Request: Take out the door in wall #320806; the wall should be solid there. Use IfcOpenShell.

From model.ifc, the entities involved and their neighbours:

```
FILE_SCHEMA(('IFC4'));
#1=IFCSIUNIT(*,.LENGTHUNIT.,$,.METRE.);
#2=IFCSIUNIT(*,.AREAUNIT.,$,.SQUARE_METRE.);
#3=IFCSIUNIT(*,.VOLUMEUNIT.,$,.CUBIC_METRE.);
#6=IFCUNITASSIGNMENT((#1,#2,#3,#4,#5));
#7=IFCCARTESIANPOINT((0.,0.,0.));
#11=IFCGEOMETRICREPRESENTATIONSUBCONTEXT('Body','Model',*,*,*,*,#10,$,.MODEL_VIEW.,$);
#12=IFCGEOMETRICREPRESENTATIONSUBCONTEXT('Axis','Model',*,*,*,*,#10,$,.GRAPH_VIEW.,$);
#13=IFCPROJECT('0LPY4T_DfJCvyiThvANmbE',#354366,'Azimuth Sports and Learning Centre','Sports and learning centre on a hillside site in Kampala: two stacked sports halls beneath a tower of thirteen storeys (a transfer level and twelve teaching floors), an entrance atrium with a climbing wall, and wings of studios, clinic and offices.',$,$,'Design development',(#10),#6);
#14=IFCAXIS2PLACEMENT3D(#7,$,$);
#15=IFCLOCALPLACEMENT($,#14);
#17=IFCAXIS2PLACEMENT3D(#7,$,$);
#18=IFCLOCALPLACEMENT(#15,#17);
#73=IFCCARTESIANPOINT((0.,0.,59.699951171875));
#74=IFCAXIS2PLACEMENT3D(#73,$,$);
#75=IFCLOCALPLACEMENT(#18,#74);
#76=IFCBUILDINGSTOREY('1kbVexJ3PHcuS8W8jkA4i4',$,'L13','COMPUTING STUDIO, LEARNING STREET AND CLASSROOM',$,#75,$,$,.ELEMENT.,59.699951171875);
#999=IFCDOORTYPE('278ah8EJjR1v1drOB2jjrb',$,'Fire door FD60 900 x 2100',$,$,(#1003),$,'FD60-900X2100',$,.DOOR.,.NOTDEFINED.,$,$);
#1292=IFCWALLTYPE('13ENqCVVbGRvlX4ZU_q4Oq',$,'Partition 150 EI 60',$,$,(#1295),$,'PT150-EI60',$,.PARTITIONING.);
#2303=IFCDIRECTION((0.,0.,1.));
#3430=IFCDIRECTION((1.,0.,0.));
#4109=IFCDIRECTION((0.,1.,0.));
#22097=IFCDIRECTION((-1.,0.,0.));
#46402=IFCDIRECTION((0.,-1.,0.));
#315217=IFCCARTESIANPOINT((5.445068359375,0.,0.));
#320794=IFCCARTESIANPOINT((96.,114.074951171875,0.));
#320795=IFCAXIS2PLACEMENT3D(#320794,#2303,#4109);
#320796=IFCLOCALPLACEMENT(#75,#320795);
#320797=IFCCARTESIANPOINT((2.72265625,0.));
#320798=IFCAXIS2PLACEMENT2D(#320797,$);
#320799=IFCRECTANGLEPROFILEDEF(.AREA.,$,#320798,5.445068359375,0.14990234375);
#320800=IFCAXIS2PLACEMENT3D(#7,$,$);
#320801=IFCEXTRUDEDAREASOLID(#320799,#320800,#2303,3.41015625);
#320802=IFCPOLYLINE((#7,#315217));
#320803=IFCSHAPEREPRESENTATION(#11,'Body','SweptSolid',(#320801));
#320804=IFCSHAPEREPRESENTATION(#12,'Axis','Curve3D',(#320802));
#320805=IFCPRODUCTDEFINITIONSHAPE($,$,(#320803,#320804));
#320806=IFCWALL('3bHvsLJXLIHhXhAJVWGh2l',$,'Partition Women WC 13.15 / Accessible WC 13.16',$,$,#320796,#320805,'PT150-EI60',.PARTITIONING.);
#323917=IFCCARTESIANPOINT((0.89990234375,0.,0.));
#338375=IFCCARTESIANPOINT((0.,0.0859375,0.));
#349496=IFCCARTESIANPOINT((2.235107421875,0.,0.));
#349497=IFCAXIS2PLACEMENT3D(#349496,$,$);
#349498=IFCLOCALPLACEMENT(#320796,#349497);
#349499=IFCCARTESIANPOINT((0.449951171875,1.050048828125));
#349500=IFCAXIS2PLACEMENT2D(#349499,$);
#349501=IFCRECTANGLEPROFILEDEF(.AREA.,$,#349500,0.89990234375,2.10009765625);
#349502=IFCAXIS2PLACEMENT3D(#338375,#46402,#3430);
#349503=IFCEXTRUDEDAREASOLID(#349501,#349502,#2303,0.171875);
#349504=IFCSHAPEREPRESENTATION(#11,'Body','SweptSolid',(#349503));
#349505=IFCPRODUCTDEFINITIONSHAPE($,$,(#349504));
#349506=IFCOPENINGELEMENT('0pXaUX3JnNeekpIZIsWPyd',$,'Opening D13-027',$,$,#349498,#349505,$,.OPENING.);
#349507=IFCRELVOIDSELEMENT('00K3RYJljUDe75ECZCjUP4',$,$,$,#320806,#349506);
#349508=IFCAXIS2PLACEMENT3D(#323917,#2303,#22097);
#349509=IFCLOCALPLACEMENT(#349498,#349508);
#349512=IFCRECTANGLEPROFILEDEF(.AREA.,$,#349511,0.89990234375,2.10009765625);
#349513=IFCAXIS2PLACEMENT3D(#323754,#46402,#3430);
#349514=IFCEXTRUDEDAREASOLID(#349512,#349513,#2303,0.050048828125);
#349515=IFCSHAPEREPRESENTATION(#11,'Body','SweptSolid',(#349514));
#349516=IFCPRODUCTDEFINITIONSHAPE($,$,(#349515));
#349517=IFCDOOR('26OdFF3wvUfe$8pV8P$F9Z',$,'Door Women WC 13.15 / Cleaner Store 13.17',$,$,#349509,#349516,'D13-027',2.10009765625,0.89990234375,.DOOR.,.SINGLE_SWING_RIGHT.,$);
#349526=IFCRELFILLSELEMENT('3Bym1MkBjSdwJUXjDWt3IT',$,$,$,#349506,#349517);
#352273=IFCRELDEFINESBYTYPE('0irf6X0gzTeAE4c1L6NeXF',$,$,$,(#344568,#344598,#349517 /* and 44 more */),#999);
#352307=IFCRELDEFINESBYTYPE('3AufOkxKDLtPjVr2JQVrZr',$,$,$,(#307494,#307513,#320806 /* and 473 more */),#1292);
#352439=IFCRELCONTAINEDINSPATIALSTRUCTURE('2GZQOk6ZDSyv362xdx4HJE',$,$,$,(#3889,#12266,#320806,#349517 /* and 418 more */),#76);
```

```python
import ifcopenshell
import ifcopenshell.api.feature
import ifcopenshell.api.root
import ifcopenshell.geom
import ifcopenshell.util.shape

model = ifcopenshell.open("model.ifc")
settings = ifcopenshell.geom.settings()


def volume(element):
    """Net volume in cubic metres, openings subtracted."""
    shape = ifcopenshell.geom.create_shape(settings, element)
    return ifcopenshell.util.shape.get_volume(shape.geometry)


door = model.by_guid("26OdFF3wvUfe$8pV8P$F9Z")
opening = door.FillsVoids[0].RelatingOpeningElement
wall = opening.VoidsElements[0].RelatingBuildingElement
before = volume(wall)

ifcopenshell.api.root.remove_product(model, product=door)
ifcopenshell.api.feature.remove_feature(model, feature=opening)

after = volume(wall)

print(f"wall volume {before:.3f} -> {after:.3f} m3")

model.write("model_updated.ifc")
```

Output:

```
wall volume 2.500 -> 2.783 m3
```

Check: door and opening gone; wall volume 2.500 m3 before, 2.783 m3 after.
